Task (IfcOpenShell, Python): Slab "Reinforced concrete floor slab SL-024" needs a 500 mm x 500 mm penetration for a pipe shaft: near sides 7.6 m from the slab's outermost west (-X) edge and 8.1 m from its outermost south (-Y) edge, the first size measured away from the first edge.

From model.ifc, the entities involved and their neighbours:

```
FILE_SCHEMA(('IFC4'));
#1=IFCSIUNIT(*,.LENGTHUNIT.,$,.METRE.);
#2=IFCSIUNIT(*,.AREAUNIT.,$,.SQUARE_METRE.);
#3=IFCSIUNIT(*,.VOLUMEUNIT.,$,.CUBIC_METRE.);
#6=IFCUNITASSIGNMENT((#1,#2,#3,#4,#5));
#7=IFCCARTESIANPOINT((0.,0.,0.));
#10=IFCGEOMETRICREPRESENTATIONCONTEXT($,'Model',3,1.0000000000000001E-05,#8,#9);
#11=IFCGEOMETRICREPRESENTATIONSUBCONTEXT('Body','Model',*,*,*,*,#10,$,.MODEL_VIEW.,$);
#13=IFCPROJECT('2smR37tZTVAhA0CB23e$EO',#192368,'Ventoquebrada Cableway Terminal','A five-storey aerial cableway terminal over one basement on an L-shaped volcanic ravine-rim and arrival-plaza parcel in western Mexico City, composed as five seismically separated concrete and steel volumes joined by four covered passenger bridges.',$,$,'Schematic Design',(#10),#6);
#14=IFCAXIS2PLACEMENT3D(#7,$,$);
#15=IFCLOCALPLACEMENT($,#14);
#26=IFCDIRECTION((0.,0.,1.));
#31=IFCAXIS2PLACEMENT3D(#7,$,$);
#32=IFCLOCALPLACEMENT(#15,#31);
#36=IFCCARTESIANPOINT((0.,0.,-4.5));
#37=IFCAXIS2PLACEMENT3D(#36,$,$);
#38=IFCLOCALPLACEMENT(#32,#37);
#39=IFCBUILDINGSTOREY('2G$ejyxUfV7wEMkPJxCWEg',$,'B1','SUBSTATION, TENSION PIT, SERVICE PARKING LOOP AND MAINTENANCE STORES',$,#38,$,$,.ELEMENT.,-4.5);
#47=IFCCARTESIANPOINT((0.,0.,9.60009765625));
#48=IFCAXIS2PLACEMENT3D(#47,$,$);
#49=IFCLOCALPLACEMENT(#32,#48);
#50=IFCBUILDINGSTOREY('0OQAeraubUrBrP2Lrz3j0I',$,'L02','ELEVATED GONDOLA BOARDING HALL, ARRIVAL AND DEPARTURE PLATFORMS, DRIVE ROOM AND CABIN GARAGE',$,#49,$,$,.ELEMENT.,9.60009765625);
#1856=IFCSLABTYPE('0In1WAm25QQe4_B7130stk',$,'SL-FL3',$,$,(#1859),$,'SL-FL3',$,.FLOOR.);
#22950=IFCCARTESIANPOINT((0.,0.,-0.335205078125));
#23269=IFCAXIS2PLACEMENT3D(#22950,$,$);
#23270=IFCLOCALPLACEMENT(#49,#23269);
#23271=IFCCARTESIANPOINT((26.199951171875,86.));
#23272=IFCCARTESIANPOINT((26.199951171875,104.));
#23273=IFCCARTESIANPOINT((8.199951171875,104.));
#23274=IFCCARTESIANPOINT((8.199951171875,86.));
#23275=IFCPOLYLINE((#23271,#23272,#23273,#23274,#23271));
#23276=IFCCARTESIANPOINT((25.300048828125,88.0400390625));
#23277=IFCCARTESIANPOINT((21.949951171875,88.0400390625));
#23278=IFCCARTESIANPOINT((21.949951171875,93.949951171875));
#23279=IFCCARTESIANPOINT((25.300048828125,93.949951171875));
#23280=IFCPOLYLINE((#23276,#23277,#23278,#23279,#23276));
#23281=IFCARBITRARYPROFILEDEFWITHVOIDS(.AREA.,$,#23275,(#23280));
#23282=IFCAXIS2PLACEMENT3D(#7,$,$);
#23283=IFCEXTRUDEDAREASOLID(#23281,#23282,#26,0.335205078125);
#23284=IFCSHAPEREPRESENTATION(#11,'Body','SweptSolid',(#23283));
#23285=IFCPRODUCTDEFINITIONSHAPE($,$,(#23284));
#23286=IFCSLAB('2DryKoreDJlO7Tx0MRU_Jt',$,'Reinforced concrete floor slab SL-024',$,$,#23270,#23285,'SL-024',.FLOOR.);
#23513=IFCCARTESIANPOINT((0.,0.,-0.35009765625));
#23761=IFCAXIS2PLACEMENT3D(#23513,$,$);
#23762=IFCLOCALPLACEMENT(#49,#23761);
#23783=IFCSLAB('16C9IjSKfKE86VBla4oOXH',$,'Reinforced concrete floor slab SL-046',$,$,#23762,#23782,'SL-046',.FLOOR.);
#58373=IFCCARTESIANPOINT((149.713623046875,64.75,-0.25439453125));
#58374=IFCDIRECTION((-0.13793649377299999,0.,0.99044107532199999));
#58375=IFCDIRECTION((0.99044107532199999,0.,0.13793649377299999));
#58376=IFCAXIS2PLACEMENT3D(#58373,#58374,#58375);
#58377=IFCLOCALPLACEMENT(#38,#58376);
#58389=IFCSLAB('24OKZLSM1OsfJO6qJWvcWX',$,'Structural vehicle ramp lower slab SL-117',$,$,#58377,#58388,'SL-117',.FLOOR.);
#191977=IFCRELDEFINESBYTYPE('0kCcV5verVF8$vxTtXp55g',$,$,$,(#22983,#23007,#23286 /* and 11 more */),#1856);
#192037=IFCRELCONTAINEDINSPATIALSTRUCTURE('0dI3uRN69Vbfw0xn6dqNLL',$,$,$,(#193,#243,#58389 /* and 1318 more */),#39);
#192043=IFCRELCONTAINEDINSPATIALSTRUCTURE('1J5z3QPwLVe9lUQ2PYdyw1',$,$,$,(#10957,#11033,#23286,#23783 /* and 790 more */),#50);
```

```python
import numpy as np
import ifcopenshell
import ifcopenshell.api.feature
import ifcopenshell.api.geometry
import ifcopenshell.api.root
import ifcopenshell.geom
import ifcopenshell.util.placement
import ifcopenshell.util.representation
import ifcopenshell.util.shape
import ifcopenshell.util.unit

model = ifcopenshell.open("model.ifc")
unit_scale = ifcopenshell.util.unit.calculate_unit_scale(model)
settings = ifcopenshell.geom.settings()


def volume(element):
    """Net volume in cubic metres, openings subtracted."""
    shape = ifcopenshell.geom.create_shape(settings, element)
    return ifcopenshell.util.shape.get_volume(shape.geometry)


slab = model.by_id(23286)
before = volume(slab)

# Extent in the slab's own axes, in metres. The edges named are its -X and -Y sides.
slab_shape = ifcopenshell.geom.create_shape(settings, slab)
vertices = ifcopenshell.util.shape.get_vertices(slab_shape.geometry)
x_min, y_min, bottom = vertices.min(axis=0)
top = vertices[:, 2].max()

opening = ifcopenshell.api.root.create_entity(model, ifc_class="IfcOpeningElement", name="Pipe shaft opening", predefined_type="OPENING")
context = ifcopenshell.util.representation.get_context(model, "Model", "Body", "MODEL_VIEW")
width, depth = 0.5, 0.5
outline = [(0.0, 0.0), (width, 0.0), (width, depth), (0.0, depth), (0.0, 0.0)]
# Overshoot both faces by 50 mm so the cut is clean.
shape = ifcopenshell.api.geometry.add_slab_representation(
    model, context=context, depth=top - bottom + 0.1, polyline=outline
)
ifcopenshell.api.geometry.assign_representation(model, product=opening, representation=shape)

matrix = ifcopenshell.util.placement.get_local_placement(slab.ObjectPlacement)
matrix[:, 3] = matrix @ np.append(np.array([x_min + 7.6, y_min + 8.1, bottom - 0.05]) / unit_scale, 1.0)
ifcopenshell.api.geometry.edit_object_placement(model, product=opening, matrix=matrix, is_si=False)
ifcopenshell.api.feature.add_feature(model, feature=opening, element=slab)

after = volume(slab)

print(f"slab volume {before:.3f} -> {after:.3f} m3")

model.write("model-out.ifc")
```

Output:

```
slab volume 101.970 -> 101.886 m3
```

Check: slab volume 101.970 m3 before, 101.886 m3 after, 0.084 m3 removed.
